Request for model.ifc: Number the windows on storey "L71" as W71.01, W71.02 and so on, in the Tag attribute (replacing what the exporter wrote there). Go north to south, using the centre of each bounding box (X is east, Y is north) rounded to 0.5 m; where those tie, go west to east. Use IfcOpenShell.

First a look at what the model holds.

```python
import ifcopenshell
import ifcopenshell.util.element
import ifcopenshell.util.placement

model = ifcopenshell.open("model.ifc")
print(model.schema)
storey = next(s for s in model.by_type("IfcBuildingStorey") if s.Name == "L71")
windows = [e for e in ifcopenshell.util.element.get_decomposition(storey) if e.is_a("IfcWindow")]
for e in sorted(windows, key=lambda e: e.id()):
    origin = ifcopenshell.util.placement.get_local_placement(e.ObjectPlacement)[:3, 3]
    print(e.id(), e.Tag, e.Name, origin.round(2) + 0.0, sep=" | ")
```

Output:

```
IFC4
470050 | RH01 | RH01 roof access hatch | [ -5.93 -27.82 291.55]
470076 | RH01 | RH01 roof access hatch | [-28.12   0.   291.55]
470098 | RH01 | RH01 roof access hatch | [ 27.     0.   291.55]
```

```python
import ifcopenshell
import ifcopenshell.geom
import ifcopenshell.util.element
import ifcopenshell.util.shape

model = ifcopenshell.open("model.ifc")
settings = ifcopenshell.geom.settings()
settings.set("use-world-coords", True)


def centre(element):
    shape = ifcopenshell.geom.create_shape(settings, element)
    return ifcopenshell.util.shape.get_bbox_centroid(shape.geometry)


storey = next(s for s in model.by_type("IfcBuildingStorey") if s.Name == "L71")
windows = [e for e in ifcopenshell.util.element.get_decomposition(storey) if e.is_a("IfcWindow")]

# Insertion points can sit at a corner or the storey origin, so sort by the geometry (in metres).
centres = {e: centre(e) for e in windows}
windows.sort(key=lambda e: (-round(centres[e][1] / 0.5), centres[e][0]))

for i, e in enumerate(windows, start=1):
    number = f"W71.{i:02d}"
    e.Tag = number
    print(e.id(), number)

model.write("model_edited.ifc")
```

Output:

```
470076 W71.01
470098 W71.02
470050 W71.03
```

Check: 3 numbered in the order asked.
